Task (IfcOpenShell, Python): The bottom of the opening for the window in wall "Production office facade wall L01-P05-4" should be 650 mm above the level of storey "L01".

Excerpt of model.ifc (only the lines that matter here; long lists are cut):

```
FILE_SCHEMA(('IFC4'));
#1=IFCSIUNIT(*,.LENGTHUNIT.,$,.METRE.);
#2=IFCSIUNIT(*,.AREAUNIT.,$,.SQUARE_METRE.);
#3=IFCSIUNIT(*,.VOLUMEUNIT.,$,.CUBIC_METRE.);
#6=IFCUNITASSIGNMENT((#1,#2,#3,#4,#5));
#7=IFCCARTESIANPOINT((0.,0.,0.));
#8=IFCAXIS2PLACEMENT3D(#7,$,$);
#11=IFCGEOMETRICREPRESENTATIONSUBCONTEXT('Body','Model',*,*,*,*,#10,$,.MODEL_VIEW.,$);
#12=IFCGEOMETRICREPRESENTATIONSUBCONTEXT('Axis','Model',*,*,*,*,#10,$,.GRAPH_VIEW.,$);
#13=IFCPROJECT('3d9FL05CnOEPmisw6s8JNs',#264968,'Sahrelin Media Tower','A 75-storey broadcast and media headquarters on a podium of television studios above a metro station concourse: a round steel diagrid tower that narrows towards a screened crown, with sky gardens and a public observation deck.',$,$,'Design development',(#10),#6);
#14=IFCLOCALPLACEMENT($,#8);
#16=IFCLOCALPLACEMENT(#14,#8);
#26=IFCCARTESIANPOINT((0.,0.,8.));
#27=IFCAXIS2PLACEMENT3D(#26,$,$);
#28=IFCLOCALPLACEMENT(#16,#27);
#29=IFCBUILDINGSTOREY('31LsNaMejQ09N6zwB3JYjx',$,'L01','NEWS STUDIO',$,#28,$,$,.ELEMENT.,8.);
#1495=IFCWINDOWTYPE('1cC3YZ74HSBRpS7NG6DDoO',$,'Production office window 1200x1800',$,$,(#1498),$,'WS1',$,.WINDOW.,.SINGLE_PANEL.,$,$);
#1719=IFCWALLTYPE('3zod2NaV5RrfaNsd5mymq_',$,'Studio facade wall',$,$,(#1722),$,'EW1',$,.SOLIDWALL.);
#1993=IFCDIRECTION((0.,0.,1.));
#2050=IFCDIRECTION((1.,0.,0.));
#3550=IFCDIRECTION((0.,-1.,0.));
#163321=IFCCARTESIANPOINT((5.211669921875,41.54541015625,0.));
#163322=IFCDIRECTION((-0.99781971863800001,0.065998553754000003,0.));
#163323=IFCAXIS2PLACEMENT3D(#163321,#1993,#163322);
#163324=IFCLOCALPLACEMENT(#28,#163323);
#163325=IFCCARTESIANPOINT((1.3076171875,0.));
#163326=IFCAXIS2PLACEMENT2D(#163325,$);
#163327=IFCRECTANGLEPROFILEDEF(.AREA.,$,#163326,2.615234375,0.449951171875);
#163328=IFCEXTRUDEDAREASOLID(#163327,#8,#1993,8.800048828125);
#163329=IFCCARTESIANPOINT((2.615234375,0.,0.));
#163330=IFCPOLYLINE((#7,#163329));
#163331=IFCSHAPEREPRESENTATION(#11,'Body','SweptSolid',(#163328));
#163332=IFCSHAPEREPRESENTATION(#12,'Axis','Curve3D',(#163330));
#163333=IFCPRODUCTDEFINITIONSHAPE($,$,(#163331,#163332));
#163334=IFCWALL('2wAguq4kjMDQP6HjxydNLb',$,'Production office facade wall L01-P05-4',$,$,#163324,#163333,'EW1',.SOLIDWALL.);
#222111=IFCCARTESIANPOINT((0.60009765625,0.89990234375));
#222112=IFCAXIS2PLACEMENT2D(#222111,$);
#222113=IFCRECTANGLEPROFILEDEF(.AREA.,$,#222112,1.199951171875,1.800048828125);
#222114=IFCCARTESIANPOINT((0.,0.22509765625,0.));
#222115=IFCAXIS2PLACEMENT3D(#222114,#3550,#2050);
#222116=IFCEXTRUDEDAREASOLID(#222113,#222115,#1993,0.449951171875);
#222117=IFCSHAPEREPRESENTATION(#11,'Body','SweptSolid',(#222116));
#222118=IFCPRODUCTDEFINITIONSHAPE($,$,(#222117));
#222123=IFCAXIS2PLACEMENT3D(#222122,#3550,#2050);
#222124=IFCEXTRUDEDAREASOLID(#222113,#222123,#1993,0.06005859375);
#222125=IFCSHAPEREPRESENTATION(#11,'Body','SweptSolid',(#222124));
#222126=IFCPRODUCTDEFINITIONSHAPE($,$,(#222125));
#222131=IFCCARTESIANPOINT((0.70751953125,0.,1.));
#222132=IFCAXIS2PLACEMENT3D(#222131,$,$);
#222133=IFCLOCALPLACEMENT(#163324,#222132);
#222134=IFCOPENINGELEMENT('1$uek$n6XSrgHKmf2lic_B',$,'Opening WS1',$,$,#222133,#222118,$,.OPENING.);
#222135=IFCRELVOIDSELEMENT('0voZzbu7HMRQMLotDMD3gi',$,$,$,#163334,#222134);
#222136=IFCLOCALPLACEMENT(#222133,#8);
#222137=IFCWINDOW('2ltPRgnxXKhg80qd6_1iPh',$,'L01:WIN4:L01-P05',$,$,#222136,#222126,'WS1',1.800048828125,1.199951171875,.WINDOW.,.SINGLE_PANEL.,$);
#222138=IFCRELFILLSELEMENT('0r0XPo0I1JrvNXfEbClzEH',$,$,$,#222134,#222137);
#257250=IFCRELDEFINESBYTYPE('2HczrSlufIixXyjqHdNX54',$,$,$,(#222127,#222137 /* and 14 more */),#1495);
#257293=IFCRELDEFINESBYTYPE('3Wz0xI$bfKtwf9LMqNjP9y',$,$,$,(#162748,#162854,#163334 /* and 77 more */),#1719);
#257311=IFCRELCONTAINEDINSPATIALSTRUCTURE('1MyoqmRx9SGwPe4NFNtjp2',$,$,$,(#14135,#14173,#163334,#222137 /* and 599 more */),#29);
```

```python
import numpy as np
import ifcopenshell
import ifcopenshell.api.geometry
import ifcopenshell.geom
import ifcopenshell.util.element
import ifcopenshell.util.placement
import ifcopenshell.util.shape
import ifcopenshell.util.unit

model = ifcopenshell.open("model.ifc")
unit_scale = ifcopenshell.util.unit.calculate_unit_scale(model)

window = model.by_guid("2ltPRgnxXKhg80qd6_1iPh")
opening = window.FillsVoids[0].RelatingOpeningElement
storey = ifcopenshell.util.element.get_container(window, ifc_class="IfcBuildingStorey")
level = ifcopenshell.util.placement.get_local_placement(storey.ObjectPlacement)[2, 3]

# The opening's origin need not be at the sill, so measure its lowest point.
shape = ifcopenshell.geom.create_shape(ifcopenshell.geom.settings(), opening)
bottom = ifcopenshell.util.shape.get_shape_bottom_elevation(shape, shape.geometry) / unit_scale
dz = level + 0.65 / unit_scale - bottom

shift = np.array([0.0, 0.0, dz])
# The window is placed relative to its opening, so it follows when the opening moves.
matrix = ifcopenshell.util.placement.get_local_placement(opening.ObjectPlacement)
matrix[:3, 3] += shift
ifcopenshell.api.geometry.edit_object_placement(
    model, product=opening, matrix=matrix, is_si=False, should_transform_children=True
)

print(f"moved by {dz * unit_scale:+.3f} m")

model.write("model_v2.ifc")
```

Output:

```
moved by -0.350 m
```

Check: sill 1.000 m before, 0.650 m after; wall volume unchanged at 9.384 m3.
